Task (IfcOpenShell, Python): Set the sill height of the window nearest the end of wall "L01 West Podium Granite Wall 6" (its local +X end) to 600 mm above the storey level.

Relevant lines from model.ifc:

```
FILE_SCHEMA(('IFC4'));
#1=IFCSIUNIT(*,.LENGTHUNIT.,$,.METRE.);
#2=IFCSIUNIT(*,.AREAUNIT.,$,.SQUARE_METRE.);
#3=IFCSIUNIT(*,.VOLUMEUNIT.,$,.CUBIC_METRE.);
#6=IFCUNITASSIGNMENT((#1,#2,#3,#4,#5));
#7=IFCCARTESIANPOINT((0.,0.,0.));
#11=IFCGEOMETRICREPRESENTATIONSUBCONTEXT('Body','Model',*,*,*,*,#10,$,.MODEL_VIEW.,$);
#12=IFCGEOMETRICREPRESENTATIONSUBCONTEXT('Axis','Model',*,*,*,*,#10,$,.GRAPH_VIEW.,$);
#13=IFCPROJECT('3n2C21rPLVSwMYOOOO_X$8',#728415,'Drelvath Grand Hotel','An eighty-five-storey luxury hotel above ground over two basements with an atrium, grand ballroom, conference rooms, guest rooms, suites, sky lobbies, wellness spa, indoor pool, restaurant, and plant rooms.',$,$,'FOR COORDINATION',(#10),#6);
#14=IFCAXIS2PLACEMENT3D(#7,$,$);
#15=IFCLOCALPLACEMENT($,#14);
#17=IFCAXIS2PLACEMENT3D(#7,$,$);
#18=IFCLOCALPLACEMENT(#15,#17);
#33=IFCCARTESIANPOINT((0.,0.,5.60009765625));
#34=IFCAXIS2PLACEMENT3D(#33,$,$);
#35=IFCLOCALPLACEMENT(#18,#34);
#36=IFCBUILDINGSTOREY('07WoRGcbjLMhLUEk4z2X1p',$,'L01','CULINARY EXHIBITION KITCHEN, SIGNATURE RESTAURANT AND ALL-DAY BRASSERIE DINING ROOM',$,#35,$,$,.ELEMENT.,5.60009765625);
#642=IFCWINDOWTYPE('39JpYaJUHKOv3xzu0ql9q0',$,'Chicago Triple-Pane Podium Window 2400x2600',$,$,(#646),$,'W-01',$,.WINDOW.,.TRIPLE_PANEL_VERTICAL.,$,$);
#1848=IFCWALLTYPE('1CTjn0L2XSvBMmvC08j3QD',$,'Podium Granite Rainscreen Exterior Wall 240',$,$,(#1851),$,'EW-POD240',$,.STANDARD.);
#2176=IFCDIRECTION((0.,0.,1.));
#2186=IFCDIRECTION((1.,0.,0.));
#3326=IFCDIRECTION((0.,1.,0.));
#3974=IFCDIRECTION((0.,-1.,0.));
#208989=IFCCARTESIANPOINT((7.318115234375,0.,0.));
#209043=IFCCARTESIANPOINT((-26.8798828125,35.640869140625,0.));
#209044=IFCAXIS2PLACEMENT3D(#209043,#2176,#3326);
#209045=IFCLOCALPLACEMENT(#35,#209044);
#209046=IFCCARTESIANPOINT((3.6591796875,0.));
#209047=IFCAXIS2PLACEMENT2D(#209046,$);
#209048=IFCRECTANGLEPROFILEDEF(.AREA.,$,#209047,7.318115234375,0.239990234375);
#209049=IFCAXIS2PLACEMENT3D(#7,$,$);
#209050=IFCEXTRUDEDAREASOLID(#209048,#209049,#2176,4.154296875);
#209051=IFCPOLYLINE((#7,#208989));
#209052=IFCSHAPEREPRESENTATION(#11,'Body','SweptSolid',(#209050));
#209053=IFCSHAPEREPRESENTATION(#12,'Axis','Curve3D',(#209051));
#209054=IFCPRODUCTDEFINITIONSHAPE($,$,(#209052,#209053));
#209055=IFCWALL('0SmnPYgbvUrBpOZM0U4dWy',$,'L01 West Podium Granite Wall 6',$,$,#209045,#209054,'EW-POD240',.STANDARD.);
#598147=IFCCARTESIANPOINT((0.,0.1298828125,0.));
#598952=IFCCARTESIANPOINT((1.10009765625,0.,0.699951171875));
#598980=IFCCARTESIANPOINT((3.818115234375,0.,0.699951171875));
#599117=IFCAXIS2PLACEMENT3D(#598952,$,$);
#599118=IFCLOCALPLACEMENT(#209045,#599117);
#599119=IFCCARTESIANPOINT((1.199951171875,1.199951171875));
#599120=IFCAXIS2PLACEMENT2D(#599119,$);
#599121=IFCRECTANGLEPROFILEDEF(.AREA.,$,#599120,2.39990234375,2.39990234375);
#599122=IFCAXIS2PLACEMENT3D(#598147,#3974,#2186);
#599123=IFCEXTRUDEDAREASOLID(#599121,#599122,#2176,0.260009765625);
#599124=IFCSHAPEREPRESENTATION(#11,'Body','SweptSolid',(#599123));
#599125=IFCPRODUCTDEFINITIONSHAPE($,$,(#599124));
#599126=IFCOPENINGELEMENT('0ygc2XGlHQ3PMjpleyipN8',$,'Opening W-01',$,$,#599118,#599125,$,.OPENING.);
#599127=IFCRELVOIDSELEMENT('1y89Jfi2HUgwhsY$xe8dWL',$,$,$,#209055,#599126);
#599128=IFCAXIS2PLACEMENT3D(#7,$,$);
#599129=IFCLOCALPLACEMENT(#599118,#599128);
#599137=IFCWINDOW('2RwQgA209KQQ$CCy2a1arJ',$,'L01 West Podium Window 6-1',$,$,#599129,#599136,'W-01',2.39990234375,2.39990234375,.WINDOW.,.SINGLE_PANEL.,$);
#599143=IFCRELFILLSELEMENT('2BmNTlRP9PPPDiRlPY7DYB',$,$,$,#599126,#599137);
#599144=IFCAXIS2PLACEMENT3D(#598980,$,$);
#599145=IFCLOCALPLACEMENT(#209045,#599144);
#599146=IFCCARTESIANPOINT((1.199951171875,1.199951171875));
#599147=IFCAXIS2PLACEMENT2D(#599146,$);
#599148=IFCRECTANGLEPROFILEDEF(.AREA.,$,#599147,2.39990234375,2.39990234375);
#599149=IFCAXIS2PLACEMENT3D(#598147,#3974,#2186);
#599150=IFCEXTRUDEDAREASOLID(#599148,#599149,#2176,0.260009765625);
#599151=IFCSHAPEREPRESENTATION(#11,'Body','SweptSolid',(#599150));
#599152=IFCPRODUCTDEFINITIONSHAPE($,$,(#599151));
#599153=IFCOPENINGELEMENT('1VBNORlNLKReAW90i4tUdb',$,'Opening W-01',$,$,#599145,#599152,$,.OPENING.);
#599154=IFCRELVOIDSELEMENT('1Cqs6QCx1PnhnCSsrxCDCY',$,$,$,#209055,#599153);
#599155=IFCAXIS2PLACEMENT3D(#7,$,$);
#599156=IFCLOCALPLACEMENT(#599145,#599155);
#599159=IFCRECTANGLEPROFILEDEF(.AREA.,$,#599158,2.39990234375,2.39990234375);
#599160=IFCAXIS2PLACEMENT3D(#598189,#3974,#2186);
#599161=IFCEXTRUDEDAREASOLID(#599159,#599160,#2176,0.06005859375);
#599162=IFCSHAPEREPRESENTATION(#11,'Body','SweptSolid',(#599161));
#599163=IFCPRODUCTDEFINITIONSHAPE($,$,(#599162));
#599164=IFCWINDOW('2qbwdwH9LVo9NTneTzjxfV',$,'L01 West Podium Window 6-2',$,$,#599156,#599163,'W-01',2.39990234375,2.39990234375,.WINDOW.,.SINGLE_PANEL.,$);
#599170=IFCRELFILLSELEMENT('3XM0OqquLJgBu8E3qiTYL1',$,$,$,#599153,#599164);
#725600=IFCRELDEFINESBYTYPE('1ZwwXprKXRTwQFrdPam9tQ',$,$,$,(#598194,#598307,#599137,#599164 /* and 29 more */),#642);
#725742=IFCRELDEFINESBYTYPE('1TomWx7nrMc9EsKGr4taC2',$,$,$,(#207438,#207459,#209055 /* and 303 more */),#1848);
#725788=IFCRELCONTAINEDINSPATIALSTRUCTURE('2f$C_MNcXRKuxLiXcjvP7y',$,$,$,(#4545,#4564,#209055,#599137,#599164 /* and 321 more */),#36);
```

```python
import numpy as np
import ifcopenshell
import ifcopenshell.api.geometry
import ifcopenshell.geom
import ifcopenshell.util.element
import ifcopenshell.util.placement
import ifcopenshell.util.shape
import ifcopenshell.util.unit

model = ifcopenshell.open("model.ifc")
unit_scale = ifcopenshell.util.unit.calculate_unit_scale(model)

window = model.by_guid("2qbwdwH9LVo9NTneTzjxfV")
opening = window.FillsVoids[0].RelatingOpeningElement
storey = ifcopenshell.util.element.get_container(window, ifc_class="IfcBuildingStorey")
level = ifcopenshell.util.placement.get_local_placement(storey.ObjectPlacement)[2, 3]

# The opening's origin need not be at the sill, so measure its lowest point.
shape = ifcopenshell.geom.create_shape(ifcopenshell.geom.settings(), opening)
bottom = ifcopenshell.util.shape.get_shape_bottom_elevation(shape, shape.geometry) / unit_scale
dz = level + 0.6 - bottom

shift = np.array([0.0, 0.0, dz])
# The window is placed relative to its opening, so it follows when the opening moves.
matrix = ifcopenshell.util.placement.get_local_placement(opening.ObjectPlacement)
matrix[:3, 3] += shift
ifcopenshell.api.geometry.edit_object_placement(
    model, product=opening, matrix=matrix, is_si=False, should_transform_children=True
)

print(f"moved by {dz * unit_scale:+.3f} m")

model.write("model_edited.ifc")
```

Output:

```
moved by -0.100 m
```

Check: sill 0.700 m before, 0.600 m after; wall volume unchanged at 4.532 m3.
